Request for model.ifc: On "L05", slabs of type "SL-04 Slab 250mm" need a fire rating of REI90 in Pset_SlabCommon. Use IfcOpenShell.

First a look at what the model holds.

```python
import ifcopenshell
import ifcopenshell.util.element

model = ifcopenshell.open("model.ifc")
print(model.schema)
storey = next(s for s in model.by_type("IfcBuildingStorey") if s.Name == "L05")
slabs = [e for e in ifcopenshell.util.element.get_decomposition(storey) if e.is_a("IfcSlab")]
seen = {}
for e in slabs:
    element_type = ifcopenshell.util.element.get_type(e)
    key = (element_type.Name if element_type != e and element_type else None, ifcopenshell.util.element.get_pset(e, "Pset_SlabCommon", "FireRating"))
    seen[key] = seen.get(key, 0) + 1
for (name, value), count in sorted(seen.items(), key=str):
    print(count, "x", name, "|", value)
```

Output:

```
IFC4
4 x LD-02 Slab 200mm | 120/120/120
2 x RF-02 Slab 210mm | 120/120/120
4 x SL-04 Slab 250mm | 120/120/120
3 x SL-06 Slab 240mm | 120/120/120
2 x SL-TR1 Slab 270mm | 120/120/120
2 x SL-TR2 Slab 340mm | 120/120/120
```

```python
import ifcopenshell
import ifcopenshell.api.pset
import ifcopenshell.util.element

model = ifcopenshell.open("model.ifc")

storey = next(s for s in model.by_type("IfcBuildingStorey") if s.Name == "L05")
slabs = [e for e in ifcopenshell.util.element.get_decomposition(storey) if e.is_a("IfcSlab")]

count = 0
for e in slabs:
    element_type = ifcopenshell.util.element.get_type(e)
    if element_type in (None, e) or element_type.Name != "SL-04 Slab 250mm":
        continue
    # add_pset returns the element's existing set when there is one.
    pset = ifcopenshell.api.pset.add_pset(model, product=e, name="Pset_SlabCommon")
    ifcopenshell.api.pset.edit_pset(model, pset=pset, properties={"FireRating": "REI90"})
    count += 1

print(count, "slabs updated")

model.write("model_rev.ifc")
```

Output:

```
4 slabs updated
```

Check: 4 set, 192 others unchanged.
